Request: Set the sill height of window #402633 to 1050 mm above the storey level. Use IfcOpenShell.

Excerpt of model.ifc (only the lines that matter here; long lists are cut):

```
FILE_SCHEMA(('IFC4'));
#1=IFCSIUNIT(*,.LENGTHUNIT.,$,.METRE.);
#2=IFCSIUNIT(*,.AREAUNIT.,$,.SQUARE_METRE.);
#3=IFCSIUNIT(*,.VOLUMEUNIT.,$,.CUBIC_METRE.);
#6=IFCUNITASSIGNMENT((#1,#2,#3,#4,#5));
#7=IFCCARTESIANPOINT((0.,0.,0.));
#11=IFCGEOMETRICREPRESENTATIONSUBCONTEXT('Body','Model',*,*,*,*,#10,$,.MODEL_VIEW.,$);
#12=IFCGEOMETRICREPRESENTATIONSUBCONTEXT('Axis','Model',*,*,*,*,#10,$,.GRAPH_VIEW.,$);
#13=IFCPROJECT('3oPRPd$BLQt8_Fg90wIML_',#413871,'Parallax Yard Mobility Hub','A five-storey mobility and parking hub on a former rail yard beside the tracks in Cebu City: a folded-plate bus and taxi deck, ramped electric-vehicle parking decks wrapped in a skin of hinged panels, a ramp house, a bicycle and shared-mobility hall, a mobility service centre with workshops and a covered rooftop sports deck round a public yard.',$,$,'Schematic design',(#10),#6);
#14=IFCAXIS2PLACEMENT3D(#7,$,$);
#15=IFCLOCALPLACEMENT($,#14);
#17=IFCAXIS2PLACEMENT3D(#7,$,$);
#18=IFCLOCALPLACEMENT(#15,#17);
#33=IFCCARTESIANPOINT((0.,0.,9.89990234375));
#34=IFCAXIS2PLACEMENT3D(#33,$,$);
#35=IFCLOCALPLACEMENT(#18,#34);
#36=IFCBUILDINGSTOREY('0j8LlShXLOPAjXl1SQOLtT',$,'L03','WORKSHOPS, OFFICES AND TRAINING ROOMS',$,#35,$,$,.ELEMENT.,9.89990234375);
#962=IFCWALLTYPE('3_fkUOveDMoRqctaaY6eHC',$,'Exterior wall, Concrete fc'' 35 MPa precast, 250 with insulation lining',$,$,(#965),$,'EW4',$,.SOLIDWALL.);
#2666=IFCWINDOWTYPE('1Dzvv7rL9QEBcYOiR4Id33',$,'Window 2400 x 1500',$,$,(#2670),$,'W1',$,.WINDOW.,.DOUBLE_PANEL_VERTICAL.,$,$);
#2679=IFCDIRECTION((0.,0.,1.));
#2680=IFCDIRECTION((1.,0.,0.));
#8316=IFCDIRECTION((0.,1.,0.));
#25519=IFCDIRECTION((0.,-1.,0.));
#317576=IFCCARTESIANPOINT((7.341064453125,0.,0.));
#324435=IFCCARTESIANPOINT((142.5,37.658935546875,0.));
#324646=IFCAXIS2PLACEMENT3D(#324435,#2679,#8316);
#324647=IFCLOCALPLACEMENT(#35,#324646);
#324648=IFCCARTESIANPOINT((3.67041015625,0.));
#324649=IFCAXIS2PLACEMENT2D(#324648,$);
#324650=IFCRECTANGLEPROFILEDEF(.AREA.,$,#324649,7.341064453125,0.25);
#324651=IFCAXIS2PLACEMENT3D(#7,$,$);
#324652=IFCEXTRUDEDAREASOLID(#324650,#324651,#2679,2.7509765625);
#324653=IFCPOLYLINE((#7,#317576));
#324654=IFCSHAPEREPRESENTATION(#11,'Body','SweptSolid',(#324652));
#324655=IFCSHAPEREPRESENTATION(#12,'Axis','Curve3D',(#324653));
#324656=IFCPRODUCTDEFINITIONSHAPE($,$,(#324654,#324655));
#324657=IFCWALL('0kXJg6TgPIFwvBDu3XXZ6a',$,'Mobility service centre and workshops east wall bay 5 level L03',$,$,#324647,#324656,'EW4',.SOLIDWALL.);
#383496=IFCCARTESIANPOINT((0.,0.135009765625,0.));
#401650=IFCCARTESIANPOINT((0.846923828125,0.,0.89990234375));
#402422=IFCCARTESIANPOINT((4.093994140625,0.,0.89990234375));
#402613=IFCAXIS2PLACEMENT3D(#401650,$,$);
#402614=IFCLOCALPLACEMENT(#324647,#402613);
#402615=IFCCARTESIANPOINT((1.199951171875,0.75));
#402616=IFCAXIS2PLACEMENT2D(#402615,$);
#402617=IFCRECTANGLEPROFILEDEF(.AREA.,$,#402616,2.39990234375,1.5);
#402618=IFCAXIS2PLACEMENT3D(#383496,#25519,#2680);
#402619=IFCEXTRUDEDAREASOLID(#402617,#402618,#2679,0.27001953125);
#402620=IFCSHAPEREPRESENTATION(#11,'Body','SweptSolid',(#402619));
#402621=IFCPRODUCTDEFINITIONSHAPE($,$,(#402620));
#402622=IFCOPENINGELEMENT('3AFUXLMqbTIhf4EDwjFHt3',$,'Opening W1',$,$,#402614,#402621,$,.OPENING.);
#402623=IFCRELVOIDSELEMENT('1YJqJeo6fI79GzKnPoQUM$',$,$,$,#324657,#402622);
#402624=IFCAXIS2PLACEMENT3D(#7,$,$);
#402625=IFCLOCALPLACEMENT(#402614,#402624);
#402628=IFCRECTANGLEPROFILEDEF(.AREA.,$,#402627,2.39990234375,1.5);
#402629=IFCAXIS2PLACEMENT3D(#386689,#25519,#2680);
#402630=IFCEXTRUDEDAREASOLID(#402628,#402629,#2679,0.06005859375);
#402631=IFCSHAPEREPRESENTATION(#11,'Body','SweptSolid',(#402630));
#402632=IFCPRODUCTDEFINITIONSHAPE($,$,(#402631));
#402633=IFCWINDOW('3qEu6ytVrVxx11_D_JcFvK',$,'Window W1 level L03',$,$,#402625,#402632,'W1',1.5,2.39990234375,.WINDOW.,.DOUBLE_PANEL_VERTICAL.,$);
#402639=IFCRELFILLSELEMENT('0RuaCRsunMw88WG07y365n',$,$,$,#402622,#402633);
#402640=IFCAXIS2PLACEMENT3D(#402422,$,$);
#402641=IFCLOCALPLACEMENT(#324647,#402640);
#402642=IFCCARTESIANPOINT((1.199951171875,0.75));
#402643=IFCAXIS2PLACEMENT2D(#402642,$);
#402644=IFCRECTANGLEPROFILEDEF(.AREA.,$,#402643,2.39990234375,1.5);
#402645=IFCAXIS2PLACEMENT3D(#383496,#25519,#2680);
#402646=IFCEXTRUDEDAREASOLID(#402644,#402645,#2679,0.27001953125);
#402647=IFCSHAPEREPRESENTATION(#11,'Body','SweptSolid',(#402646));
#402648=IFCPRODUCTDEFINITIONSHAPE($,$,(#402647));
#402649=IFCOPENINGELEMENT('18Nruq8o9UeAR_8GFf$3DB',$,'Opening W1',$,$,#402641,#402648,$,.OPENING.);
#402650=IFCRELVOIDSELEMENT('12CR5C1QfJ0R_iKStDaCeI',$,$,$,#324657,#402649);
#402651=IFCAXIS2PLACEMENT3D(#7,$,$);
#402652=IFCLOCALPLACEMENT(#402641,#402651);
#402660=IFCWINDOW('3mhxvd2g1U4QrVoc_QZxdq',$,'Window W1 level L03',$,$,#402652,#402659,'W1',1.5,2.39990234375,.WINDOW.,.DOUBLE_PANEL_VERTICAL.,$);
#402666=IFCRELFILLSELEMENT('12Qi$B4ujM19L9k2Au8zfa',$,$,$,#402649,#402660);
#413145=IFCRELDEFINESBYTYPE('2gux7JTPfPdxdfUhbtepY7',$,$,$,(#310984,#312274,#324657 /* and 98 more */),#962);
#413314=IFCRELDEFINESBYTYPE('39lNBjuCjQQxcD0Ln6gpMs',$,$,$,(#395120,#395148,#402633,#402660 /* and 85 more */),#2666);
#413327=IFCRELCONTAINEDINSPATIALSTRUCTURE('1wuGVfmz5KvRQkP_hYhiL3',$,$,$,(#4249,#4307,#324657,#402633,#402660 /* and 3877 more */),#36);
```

```python
import numpy as np
import ifcopenshell
import ifcopenshell.api.geometry
import ifcopenshell.geom
import ifcopenshell.util.element
import ifcopenshell.util.placement
import ifcopenshell.util.shape
import ifcopenshell.util.unit

model = ifcopenshell.open("model.ifc")
unit_scale = ifcopenshell.util.unit.calculate_unit_scale(model)

window = model.by_guid("3qEu6ytVrVxx11_D_JcFvK")
opening = window.FillsVoids[0].RelatingOpeningElement
storey = ifcopenshell.util.element.get_container(window, ifc_class="IfcBuildingStorey")
level = ifcopenshell.util.placement.get_local_placement(storey.ObjectPlacement)[2, 3]

# The opening's origin need not be at the sill, so measure its lowest point.
shape = ifcopenshell.geom.create_shape(ifcopenshell.geom.settings(), opening)
bottom = ifcopenshell.util.shape.get_shape_bottom_elevation(shape, shape.geometry) / unit_scale
dz = level + 1.05 - bottom

shift = np.array([0.0, 0.0, dz])
# The window is placed relative to its opening, so it follows when the opening moves.
matrix = ifcopenshell.util.placement.get_local_placement(opening.ObjectPlacement)
matrix[:3, 3] += shift
ifcopenshell.api.geometry.edit_object_placement(
    model, product=opening, matrix=matrix, is_si=False, should_transform_children=True
)

print(f"moved by {dz * unit_scale:+.3f} m")

model.write("model_edited.ifc")
```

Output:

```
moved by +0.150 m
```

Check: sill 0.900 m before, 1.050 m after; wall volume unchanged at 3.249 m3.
